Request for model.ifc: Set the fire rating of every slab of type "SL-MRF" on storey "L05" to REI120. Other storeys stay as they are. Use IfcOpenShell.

First a look at what the model holds.

```python
import ifcopenshell
import ifcopenshell.util.element

model = ifcopenshell.open("model.ifc")
print(model.schema)
storey = next(s for s in model.by_type("IfcBuildingStorey") if s.Name == "L05")
slabs = [e for e in ifcopenshell.util.element.get_decomposition(storey) if e.is_a("IfcSlab")]
seen = {}
for e in slabs:
    element_type = ifcopenshell.util.element.get_type(e)
    key = (element_type.Name if element_type != e and element_type else None, ifcopenshell.util.element.get_pset(e, "Pset_SlabCommon", "FireRating"))
    seen[key] = seen.get(key, 0) + 1
for (name, value), count in sorted(seen.items(), key=str):
    print(count, "x", name, "|", value)
```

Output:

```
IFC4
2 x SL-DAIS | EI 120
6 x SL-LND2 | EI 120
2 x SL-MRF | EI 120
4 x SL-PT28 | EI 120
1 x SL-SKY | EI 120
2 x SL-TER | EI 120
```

```python
import ifcopenshell
import ifcopenshell.api.pset
import ifcopenshell.util.element

model = ifcopenshell.open("model.ifc")

storey = next(s for s in model.by_type("IfcBuildingStorey") if s.Name == "L05")
slabs = [e for e in ifcopenshell.util.element.get_decomposition(storey) if e.is_a("IfcSlab")]

count = 0
for e in slabs:
    element_type = ifcopenshell.util.element.get_type(e)
    if element_type in (None, e) or element_type.Name != "SL-MRF":
        continue
    # add_pset returns the element's existing set when there is one.
    pset = ifcopenshell.api.pset.add_pset(model, product=e, name="Pset_SlabCommon")
    ifcopenshell.api.pset.edit_pset(model, pset=pset, properties={"FireRating": "REI120"})
    count += 1

print(count, "slabs updated")

model.write("model_updated.ifc")
```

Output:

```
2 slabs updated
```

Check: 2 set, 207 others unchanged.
